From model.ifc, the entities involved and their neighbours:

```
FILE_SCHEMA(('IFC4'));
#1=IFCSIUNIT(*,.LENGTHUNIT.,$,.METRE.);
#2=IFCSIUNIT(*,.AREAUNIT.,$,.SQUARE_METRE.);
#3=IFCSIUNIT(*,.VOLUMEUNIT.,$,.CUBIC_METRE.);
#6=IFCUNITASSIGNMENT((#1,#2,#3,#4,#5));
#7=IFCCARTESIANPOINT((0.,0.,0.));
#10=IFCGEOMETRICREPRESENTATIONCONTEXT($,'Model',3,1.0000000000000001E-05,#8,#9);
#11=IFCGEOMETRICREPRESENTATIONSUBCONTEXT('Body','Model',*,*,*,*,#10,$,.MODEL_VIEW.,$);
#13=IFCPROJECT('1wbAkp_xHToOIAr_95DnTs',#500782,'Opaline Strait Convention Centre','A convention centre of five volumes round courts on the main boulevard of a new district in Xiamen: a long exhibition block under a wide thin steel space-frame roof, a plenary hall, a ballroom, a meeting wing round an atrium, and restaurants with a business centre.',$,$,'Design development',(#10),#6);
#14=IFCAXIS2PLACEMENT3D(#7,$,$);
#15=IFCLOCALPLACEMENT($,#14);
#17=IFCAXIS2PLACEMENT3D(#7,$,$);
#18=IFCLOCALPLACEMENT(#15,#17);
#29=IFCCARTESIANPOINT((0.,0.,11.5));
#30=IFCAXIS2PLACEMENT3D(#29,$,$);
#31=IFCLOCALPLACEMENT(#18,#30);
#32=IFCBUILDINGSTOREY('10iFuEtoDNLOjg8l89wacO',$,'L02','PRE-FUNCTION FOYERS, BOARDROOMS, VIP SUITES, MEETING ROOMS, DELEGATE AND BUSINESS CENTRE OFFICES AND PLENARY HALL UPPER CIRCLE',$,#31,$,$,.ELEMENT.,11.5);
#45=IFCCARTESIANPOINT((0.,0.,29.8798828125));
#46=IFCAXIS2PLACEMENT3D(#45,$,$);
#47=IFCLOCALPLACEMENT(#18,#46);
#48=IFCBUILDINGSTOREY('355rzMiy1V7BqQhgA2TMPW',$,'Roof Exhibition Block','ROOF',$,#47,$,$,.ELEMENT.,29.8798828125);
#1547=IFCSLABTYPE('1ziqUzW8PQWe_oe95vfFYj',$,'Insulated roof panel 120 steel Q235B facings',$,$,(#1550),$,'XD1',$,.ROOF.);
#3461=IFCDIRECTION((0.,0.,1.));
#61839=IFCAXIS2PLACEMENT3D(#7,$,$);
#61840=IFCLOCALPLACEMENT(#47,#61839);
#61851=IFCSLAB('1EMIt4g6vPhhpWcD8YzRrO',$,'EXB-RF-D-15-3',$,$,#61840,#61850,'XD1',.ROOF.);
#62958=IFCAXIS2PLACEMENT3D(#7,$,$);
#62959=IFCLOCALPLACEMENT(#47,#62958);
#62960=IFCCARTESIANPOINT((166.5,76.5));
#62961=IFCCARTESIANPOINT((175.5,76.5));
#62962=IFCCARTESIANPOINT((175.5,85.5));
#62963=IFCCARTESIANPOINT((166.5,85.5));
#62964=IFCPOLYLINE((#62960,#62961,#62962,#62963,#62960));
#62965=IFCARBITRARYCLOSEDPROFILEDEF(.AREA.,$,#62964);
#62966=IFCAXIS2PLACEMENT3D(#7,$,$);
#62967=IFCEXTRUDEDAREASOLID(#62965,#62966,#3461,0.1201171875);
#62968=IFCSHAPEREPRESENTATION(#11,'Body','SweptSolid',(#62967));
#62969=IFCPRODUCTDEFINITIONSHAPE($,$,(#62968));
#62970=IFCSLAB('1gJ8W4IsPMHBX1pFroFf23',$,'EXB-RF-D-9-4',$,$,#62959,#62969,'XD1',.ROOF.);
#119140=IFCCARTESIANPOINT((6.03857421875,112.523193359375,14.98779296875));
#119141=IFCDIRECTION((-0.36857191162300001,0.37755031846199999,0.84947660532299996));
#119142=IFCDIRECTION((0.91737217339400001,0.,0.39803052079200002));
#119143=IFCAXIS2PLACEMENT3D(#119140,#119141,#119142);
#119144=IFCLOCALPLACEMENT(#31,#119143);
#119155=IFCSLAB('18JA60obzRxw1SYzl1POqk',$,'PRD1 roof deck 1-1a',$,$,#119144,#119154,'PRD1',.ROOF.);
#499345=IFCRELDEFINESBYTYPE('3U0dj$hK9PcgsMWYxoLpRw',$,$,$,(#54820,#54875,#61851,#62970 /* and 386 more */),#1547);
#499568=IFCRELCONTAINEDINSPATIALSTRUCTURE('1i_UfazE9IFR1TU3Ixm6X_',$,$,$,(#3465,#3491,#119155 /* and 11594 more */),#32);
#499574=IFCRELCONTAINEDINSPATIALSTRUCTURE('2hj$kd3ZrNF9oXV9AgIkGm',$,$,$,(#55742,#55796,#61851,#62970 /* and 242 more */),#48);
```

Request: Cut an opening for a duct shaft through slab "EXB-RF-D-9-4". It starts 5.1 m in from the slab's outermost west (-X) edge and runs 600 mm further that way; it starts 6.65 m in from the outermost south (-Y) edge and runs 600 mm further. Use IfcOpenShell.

```python
import numpy as np
import ifcopenshell
import ifcopenshell.api.feature
import ifcopenshell.api.geometry
import ifcopenshell.api.root
import ifcopenshell.geom
import ifcopenshell.util.placement
import ifcopenshell.util.representation
import ifcopenshell.util.shape
import ifcopenshell.util.unit

model = ifcopenshell.open("model.ifc")
unit_scale = ifcopenshell.util.unit.calculate_unit_scale(model)
settings = ifcopenshell.geom.settings()


def volume(element):
    """Net volume in cubic metres, openings subtracted."""
    shape = ifcopenshell.geom.create_shape(settings, element)
    return ifcopenshell.util.shape.get_volume(shape.geometry)


slab = model.by_guid("1gJ8W4IsPMHBX1pFroFf23")
before = volume(slab)

# Extent in the slab's own axes, in metres. The edges named are its -X and -Y sides.
slab_shape = ifcopenshell.geom.create_shape(settings, slab)
vertices = ifcopenshell.util.shape.get_vertices(slab_shape.geometry)
x_min, y_min, bottom = vertices.min(axis=0)
top = vertices[:, 2].max()

opening = ifcopenshell.api.root.create_entity(model, ifc_class="IfcOpeningElement", name="Duct shaft opening", predefined_type="OPENING")
context = ifcopenshell.util.representation.get_context(model, "Model", "Body", "MODEL_VIEW")
width, depth = 0.6, 0.6
outline = [(0.0, 0.0), (width, 0.0), (width, depth), (0.0, depth), (0.0, 0.0)]
# Overshoot both faces by 50 mm so the cut is clean.
shape = ifcopenshell.api.geometry.add_slab_representation(
    model, context=context, depth=top - bottom + 0.1, polyline=outline
)
ifcopenshell.api.geometry.assign_representation(model, product=opening, representation=shape)

matrix = ifcopenshell.util.placement.get_local_placement(slab.ObjectPlacement)
matrix[:, 3] = matrix @ np.append(np.array([x_min + 5.1, y_min + 6.65, bottom - 0.05]) / unit_scale, 1.0)
ifcopenshell.api.geometry.edit_object_placement(model, product=opening, matrix=matrix, is_si=False)
ifcopenshell.api.feature.add_feature(model, feature=opening, element=slab)

after = volume(slab)

print(f"slab volume {before:.3f} -> {after:.3f} m3")

model.write("model-out.ifc")
```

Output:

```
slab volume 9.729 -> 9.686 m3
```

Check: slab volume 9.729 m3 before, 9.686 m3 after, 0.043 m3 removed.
